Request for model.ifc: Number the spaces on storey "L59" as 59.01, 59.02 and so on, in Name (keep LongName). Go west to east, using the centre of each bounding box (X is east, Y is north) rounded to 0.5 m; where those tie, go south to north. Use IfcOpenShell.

First a look at what the model holds.

```python
import ifcopenshell
import ifcopenshell.util.element
import ifcopenshell.util.placement

model = ifcopenshell.open("model.ifc")
print(model.schema)
storey = next(s for s in model.by_type("IfcBuildingStorey") if s.Name == "L59")
spaces = [e for e in ifcopenshell.util.element.get_decomposition(storey) if e.is_a("IfcSpace")]
for e in sorted(spaces, key=lambda e: e.id()):
    origin = ifcopenshell.util.placement.get_local_placement(e.ObjectPlacement)[:3, 3]
    print(e.id(), e.Name, e.LongName, origin.round(2) + 0.0, sep=" | ")
```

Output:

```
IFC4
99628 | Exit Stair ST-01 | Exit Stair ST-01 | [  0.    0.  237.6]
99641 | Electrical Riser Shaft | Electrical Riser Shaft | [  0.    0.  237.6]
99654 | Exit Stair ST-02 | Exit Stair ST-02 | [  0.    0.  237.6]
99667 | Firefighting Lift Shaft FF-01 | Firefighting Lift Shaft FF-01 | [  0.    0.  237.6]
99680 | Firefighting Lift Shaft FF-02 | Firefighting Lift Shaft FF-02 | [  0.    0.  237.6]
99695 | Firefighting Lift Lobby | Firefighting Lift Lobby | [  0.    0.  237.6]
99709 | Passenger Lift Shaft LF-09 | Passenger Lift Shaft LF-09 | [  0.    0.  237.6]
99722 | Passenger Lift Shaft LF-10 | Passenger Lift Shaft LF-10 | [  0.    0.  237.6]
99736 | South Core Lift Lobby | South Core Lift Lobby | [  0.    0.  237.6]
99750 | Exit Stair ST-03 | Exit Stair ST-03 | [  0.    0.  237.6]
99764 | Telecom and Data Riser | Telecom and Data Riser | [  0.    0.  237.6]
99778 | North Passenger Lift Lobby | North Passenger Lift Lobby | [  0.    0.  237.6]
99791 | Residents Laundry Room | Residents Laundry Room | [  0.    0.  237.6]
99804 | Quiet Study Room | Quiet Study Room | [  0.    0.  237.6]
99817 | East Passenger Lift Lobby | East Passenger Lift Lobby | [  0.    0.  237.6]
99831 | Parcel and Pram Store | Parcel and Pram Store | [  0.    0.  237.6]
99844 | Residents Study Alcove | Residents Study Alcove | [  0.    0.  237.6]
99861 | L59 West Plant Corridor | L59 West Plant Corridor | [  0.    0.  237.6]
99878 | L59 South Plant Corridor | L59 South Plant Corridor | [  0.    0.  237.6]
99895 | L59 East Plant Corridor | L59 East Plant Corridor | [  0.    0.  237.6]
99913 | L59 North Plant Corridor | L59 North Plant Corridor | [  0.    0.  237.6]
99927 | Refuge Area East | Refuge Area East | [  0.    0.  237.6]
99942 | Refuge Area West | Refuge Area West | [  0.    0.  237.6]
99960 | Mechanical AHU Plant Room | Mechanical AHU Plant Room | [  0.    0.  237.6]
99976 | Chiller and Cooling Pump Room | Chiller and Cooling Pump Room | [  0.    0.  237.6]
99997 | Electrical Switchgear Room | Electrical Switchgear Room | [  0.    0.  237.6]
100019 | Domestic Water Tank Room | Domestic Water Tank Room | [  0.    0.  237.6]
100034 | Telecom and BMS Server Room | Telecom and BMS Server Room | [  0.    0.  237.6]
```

```python
import ifcopenshell
import ifcopenshell.geom
import ifcopenshell.util.element
import ifcopenshell.util.shape

model = ifcopenshell.open("model.ifc")
settings = ifcopenshell.geom.settings()
settings.set("use-world-coords", True)


def centre(element):
    shape = ifcopenshell.geom.create_shape(settings, element)
    return ifcopenshell.util.shape.get_bbox_centroid(shape.geometry)


storey = next(s for s in model.by_type("IfcBuildingStorey") if s.Name == "L59")
spaces = [e for e in ifcopenshell.util.element.get_decomposition(storey) if e.is_a("IfcSpace")]

# Insertion points can sit at a corner or the storey origin, so sort by the geometry (in metres).
centres = {e: centre(e) for e in spaces}
spaces.sort(key=lambda e: (round(centres[e][0] / 0.5), centres[e][1]))

for i, e in enumerate(spaces, start=1):
    number = f"59.{i:02d}"
    e.Name = number
    print(e.id(), number)

model.write("model_updated.ifc")
```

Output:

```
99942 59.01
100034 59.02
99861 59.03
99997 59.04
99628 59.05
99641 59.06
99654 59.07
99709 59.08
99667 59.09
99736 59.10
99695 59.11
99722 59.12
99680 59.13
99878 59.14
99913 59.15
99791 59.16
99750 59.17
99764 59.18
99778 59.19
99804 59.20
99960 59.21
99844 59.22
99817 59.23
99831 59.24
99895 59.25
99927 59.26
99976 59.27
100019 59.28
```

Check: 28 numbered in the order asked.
